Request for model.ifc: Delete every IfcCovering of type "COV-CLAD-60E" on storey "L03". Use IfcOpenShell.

First a look at what the model holds.

```python
import ifcopenshell
import ifcopenshell.util.element

model = ifcopenshell.open("model.ifc")
print(model.schema)
storey = next(s for s in model.by_type("IfcBuildingStorey") if s.Name == "L03")
coverings = [e for e in ifcopenshell.util.element.get_decomposition(storey) if e.is_a("IfcCovering")]
seen = {}
for e in coverings:
    element_type = ifcopenshell.util.element.get_type(e)
    name = element_type.Name if element_type not in (None, e) else None
    seen[name] = seen.get(name, 0) + 1
for name, count in sorted(seen.items(), key=str):
    print(count, "x", name)
```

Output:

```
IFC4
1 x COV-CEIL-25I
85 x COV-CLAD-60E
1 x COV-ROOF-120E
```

```python
import ifcopenshell
import ifcopenshell.api.root
import ifcopenshell.util.element

model = ifcopenshell.open("model.ifc")

storey = next(s for s in model.by_type("IfcBuildingStorey") if s.Name == "L03")
coverings = [e for e in ifcopenshell.util.element.get_decomposition(storey) if e.is_a("IfcCovering")]
targets = [e for e in coverings if (t := ifcopenshell.util.element.get_type(e)) not in (None, e) and t.Name == "COV-CLAD-60E"]

for e in targets:
    ifcopenshell.api.root.remove_product(model, product=e)
print(len(targets), "removed")

model.write("model_updated.ifc")
```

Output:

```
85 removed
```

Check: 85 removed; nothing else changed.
